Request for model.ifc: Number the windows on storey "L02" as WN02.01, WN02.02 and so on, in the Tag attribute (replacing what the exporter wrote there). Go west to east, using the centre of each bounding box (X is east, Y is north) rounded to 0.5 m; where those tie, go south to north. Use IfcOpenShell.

First a look at what the model holds.

```python
import ifcopenshell
import ifcopenshell.util.element
import ifcopenshell.util.placement

model = ifcopenshell.open("model.ifc")
print(model.schema)
storey = next(s for s in model.by_type("IfcBuildingStorey") if s.Name == "L02")
windows = [e for e in ifcopenshell.util.element.get_decomposition(storey) if e.is_a("IfcWindow")]
for e in sorted(windows, key=lambda e: e.id()):
    origin = ifcopenshell.util.placement.get_local_placement(e.ObjectPlacement)[:3, 3]
    print(e.id(), e.Tag, e.Name, origin.round(2) + 0.0, sep=" | ")
```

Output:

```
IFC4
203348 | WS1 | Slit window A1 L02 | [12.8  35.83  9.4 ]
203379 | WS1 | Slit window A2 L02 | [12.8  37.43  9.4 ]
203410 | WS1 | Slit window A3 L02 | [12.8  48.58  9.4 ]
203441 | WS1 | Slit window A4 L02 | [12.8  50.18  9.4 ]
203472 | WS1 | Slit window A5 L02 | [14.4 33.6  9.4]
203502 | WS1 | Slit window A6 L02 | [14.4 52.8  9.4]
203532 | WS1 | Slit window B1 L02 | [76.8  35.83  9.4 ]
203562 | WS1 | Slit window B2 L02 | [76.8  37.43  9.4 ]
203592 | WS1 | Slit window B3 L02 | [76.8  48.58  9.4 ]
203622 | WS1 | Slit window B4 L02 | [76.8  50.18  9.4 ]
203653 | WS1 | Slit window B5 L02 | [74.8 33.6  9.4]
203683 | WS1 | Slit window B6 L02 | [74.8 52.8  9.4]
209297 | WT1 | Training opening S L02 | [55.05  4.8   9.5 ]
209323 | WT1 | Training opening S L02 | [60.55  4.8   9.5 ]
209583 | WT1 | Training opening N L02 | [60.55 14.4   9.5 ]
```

```python
import ifcopenshell
import ifcopenshell.geom
import ifcopenshell.util.element
import ifcopenshell.util.shape

model = ifcopenshell.open("model.ifc")
settings = ifcopenshell.geom.settings()
settings.set("use-world-coords", True)


def centre(element):
    shape = ifcopenshell.geom.create_shape(settings, element)
    return ifcopenshell.util.shape.get_bbox_centroid(shape.geometry)


storey = next(s for s in model.by_type("IfcBuildingStorey") if s.Name == "L02")
windows = [e for e in ifcopenshell.util.element.get_decomposition(storey) if e.is_a("IfcWindow")]

# Insertion points can sit at a corner or the storey origin, so sort by the geometry (in metres).
centres = {e: centre(e) for e in windows}
windows.sort(key=lambda e: (round(centres[e][0] / 0.5), centres[e][1]))

for i, e in enumerate(windows, start=1):
    number = f"WN02.{i:02d}"
    e.Tag = number
    print(e.id(), number)

model.write("model_rev.ifc")
```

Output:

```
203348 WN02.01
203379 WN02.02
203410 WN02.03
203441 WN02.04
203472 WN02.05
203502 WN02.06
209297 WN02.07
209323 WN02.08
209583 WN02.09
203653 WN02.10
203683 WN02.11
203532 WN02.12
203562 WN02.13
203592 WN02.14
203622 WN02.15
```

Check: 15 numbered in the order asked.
